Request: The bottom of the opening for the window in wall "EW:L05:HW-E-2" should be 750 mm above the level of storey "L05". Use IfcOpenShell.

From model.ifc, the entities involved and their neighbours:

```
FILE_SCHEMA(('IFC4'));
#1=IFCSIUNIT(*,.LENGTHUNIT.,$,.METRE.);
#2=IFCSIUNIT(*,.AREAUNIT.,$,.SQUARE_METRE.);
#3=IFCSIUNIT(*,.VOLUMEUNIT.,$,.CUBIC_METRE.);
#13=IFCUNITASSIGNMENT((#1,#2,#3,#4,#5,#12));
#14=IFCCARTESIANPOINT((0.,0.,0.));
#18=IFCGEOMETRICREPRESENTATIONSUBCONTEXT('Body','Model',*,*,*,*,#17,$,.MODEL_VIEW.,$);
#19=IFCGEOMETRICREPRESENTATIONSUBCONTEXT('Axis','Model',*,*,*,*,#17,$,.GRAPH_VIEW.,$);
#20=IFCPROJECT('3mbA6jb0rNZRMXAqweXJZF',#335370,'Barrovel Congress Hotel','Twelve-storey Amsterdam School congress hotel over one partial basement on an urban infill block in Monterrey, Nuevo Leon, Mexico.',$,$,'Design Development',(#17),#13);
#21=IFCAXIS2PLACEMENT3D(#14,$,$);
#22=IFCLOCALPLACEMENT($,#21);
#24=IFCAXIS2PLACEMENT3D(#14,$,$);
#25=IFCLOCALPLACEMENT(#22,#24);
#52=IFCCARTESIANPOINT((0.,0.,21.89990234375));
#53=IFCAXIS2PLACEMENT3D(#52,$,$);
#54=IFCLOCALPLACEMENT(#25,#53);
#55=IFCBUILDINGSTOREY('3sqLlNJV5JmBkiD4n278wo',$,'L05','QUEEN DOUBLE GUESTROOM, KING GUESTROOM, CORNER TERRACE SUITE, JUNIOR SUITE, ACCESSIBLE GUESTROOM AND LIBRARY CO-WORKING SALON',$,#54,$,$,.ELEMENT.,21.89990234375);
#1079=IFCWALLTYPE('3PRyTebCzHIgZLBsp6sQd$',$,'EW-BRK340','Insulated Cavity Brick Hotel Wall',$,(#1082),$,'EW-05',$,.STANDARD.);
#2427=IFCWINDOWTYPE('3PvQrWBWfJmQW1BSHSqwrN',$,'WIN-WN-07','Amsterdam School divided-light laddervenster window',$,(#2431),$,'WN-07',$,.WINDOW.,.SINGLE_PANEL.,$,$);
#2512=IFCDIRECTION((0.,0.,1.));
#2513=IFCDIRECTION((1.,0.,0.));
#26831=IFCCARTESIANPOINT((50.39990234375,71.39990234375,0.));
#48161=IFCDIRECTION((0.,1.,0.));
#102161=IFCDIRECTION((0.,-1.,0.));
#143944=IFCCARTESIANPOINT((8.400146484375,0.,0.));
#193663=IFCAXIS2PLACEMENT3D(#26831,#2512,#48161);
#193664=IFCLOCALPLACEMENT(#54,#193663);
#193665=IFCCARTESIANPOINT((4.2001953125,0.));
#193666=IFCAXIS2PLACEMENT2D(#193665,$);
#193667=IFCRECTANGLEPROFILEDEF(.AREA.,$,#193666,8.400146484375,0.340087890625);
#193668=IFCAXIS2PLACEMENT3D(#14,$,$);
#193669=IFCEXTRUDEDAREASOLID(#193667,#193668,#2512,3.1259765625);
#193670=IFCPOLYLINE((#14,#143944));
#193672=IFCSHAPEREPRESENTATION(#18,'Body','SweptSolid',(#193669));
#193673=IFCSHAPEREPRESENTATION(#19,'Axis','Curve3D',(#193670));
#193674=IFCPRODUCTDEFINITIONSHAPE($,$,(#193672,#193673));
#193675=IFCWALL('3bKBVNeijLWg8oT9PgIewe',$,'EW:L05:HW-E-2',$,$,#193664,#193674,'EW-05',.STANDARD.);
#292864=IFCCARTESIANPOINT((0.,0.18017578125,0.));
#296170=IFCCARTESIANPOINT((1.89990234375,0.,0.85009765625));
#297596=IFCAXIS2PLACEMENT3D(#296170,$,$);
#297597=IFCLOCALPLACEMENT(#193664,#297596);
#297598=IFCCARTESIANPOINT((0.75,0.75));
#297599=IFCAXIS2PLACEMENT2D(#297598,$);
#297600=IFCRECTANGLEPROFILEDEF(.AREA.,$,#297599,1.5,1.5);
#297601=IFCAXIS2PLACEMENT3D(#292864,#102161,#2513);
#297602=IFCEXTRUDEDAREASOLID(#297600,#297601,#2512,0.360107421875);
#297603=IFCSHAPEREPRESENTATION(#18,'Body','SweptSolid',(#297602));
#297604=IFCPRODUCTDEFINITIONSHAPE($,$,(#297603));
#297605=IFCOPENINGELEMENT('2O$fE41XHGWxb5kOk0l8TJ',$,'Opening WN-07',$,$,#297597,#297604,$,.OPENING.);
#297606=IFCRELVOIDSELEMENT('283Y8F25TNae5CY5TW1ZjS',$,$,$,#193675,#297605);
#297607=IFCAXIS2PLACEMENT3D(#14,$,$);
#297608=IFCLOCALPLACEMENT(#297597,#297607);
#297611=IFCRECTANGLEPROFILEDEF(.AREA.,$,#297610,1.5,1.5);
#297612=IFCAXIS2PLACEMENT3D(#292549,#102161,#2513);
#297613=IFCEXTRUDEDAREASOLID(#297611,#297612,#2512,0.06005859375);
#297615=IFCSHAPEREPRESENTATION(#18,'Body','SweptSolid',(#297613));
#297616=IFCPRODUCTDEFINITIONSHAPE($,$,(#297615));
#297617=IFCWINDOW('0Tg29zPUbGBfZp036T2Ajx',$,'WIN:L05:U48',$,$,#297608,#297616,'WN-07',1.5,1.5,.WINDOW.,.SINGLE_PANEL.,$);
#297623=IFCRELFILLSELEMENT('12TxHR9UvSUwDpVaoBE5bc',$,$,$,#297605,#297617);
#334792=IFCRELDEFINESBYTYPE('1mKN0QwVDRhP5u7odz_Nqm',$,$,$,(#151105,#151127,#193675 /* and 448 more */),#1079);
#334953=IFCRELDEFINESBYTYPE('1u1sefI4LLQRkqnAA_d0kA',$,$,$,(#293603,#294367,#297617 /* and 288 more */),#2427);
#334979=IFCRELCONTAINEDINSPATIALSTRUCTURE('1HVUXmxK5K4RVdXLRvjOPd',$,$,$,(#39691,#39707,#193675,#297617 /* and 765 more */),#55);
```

```python
import numpy as np
import ifcopenshell
import ifcopenshell.api.geometry
import ifcopenshell.geom
import ifcopenshell.util.element
import ifcopenshell.util.placement
import ifcopenshell.util.shape
import ifcopenshell.util.unit

model = ifcopenshell.open("model.ifc")
unit_scale = ifcopenshell.util.unit.calculate_unit_scale(model)

window = model.by_guid("0Tg29zPUbGBfZp036T2Ajx")
opening = window.FillsVoids[0].RelatingOpeningElement
storey = ifcopenshell.util.element.get_container(window, ifc_class="IfcBuildingStorey")
level = ifcopenshell.util.placement.get_local_placement(storey.ObjectPlacement)[2, 3]

# The opening's origin need not be at the sill, so measure its lowest point.
shape = ifcopenshell.geom.create_shape(ifcopenshell.geom.settings(), opening)
bottom = ifcopenshell.util.shape.get_shape_bottom_elevation(shape, shape.geometry) / unit_scale
dz = level + 0.75 / unit_scale - bottom

shift = np.array([0.0, 0.0, dz])
# The window is placed relative to its opening, so it follows when the opening moves.
matrix = ifcopenshell.util.placement.get_local_placement(opening.ObjectPlacement)
matrix[:3, 3] += shift
ifcopenshell.api.geometry.edit_object_placement(
    model, product=opening, matrix=matrix, is_si=False, should_transform_children=True
)

print(f"moved by {dz * unit_scale:+.3f} m")

model.write("model_updated.ifc")
```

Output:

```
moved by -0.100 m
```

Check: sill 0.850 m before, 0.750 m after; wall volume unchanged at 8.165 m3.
